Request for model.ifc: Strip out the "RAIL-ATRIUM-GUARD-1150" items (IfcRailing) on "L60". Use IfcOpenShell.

First a look at what the model holds.

```python
import ifcopenshell
import ifcopenshell.util.element

model = ifcopenshell.open("model.ifc")
print(model.schema)
storey = next(s for s in model.by_type("IfcBuildingStorey") if s.Name == "L60")
railings = [e for e in ifcopenshell.util.element.get_decomposition(storey) if e.is_a("IfcRailing")]
seen = {}
for e in railings:
    element_type = ifcopenshell.util.element.get_type(e)
    name = element_type.Name if element_type not in (None, e) else None
    seen[name] = seen.get(name, 0) + 1
for name, count in sorted(seen.items(), key=str):
    print(count, "x", name)
```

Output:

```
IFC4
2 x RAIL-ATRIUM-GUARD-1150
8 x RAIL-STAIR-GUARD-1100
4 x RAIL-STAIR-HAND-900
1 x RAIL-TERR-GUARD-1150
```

```python
import ifcopenshell
import ifcopenshell.api.root
import ifcopenshell.util.element

model = ifcopenshell.open("model.ifc")

storey = next(s for s in model.by_type("IfcBuildingStorey") if s.Name == "L60")
railings = [e for e in ifcopenshell.util.element.get_decomposition(storey) if e.is_a("IfcRailing")]
targets = [e for e in railings if (t := ifcopenshell.util.element.get_type(e)) not in (None, e) and t.Name == "RAIL-ATRIUM-GUARD-1150"]

for e in targets:
    ifcopenshell.api.root.remove_product(model, product=e)
print(len(targets), "removed")

model.write("model_rev.ifc")
```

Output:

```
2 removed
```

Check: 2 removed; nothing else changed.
